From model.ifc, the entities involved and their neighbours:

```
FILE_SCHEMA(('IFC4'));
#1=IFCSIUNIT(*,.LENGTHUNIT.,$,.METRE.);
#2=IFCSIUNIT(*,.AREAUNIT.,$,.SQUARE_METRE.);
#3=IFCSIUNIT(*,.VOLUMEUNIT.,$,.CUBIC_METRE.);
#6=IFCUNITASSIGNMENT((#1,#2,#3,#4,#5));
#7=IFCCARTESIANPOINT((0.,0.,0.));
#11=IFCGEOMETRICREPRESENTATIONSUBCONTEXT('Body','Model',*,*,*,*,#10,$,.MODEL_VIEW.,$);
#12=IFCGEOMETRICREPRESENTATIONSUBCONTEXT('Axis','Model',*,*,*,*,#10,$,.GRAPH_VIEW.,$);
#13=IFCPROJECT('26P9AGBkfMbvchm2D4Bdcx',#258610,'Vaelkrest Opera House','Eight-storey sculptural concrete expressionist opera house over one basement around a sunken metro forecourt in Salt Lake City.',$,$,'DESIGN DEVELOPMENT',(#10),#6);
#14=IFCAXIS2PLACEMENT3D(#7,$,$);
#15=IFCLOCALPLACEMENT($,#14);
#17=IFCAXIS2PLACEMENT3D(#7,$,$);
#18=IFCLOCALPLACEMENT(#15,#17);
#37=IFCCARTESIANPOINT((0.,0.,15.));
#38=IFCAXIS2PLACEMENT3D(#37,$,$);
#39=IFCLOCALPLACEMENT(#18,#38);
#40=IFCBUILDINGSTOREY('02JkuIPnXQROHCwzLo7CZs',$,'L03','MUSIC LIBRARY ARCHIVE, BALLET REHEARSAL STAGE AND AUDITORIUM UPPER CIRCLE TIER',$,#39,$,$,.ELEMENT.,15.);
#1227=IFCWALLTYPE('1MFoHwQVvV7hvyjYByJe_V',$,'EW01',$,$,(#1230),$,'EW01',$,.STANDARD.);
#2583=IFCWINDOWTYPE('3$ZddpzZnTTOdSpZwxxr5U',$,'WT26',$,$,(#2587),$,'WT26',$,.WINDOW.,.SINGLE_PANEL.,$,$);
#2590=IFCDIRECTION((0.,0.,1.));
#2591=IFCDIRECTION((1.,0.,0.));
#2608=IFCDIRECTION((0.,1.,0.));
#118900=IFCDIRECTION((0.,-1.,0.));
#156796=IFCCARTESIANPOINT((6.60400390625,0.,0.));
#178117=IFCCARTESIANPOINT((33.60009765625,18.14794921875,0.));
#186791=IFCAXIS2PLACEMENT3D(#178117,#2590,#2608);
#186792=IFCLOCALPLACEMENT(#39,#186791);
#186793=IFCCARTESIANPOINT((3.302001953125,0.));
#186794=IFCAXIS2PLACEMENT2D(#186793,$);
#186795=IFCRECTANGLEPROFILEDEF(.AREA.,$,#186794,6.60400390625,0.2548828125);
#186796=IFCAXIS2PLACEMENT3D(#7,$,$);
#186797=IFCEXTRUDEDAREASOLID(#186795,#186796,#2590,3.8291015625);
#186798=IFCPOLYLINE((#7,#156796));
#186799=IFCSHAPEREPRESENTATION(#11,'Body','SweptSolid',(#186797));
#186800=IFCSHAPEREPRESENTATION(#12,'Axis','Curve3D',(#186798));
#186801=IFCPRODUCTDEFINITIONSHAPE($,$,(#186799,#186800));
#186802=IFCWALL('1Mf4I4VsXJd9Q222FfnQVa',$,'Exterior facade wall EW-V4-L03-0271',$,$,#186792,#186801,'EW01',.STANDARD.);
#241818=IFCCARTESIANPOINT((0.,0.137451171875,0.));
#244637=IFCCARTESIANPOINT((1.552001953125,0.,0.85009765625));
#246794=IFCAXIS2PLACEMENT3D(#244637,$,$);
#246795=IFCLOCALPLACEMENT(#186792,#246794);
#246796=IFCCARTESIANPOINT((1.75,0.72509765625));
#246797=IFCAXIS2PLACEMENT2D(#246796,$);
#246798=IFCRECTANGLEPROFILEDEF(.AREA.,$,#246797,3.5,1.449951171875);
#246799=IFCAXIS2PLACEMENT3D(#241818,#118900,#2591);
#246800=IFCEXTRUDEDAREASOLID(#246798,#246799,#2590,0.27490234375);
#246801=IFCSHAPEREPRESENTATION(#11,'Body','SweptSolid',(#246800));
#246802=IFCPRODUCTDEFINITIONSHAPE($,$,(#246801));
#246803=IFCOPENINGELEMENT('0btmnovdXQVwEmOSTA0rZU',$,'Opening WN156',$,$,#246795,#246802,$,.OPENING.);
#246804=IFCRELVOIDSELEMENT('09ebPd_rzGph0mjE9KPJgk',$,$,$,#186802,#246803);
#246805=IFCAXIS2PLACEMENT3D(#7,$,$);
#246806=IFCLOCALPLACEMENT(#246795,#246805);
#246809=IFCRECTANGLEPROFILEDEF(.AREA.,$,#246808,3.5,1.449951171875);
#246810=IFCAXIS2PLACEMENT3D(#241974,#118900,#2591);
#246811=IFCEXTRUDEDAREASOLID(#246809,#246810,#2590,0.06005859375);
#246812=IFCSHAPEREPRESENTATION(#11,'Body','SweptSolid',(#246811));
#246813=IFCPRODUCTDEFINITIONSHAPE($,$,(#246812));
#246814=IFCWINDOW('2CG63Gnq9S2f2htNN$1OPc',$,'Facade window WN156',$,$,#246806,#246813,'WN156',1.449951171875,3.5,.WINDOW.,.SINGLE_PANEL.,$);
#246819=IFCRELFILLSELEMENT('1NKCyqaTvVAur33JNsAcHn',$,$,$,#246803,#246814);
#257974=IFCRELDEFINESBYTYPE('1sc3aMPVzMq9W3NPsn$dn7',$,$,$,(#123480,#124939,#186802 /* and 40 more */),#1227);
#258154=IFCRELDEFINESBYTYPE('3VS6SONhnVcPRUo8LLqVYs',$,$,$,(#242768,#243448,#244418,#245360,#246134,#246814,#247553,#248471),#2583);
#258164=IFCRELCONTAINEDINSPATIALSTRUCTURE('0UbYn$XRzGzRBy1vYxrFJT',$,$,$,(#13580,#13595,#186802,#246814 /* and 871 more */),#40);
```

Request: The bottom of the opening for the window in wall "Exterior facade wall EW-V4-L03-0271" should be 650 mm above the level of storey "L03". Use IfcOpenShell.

```python
import numpy as np
import ifcopenshell
import ifcopenshell.api.geometry
import ifcopenshell.geom
import ifcopenshell.util.element
import ifcopenshell.util.placement
import ifcopenshell.util.shape
import ifcopenshell.util.unit

model = ifcopenshell.open("model.ifc")
unit_scale = ifcopenshell.util.unit.calculate_unit_scale(model)

window = model.by_id(246814)
opening = window.FillsVoids[0].RelatingOpeningElement
storey = ifcopenshell.util.element.get_container(window, ifc_class="IfcBuildingStorey")
level = ifcopenshell.util.placement.get_local_placement(storey.ObjectPlacement)[2, 3]

# The opening's origin need not be at the sill, so measure its lowest point.
shape = ifcopenshell.geom.create_shape(ifcopenshell.geom.settings(), opening)
bottom = ifcopenshell.util.shape.get_shape_bottom_elevation(shape, shape.geometry) / unit_scale
dz = level + 0.65 - bottom

shift = np.array([0.0, 0.0, dz])
# The window is placed relative to its opening, so it follows when the opening moves.
matrix = ifcopenshell.util.placement.get_local_placement(opening.ObjectPlacement)
matrix[:3, 3] += shift
ifcopenshell.api.geometry.edit_object_placement(
    model, product=opening, matrix=matrix, is_si=False, should_transform_children=True
)

print(f"moved by {dz * unit_scale:+.3f} m")

model.write("model_v2.ifc")
```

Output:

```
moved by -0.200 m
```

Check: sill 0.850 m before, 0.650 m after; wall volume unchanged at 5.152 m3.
